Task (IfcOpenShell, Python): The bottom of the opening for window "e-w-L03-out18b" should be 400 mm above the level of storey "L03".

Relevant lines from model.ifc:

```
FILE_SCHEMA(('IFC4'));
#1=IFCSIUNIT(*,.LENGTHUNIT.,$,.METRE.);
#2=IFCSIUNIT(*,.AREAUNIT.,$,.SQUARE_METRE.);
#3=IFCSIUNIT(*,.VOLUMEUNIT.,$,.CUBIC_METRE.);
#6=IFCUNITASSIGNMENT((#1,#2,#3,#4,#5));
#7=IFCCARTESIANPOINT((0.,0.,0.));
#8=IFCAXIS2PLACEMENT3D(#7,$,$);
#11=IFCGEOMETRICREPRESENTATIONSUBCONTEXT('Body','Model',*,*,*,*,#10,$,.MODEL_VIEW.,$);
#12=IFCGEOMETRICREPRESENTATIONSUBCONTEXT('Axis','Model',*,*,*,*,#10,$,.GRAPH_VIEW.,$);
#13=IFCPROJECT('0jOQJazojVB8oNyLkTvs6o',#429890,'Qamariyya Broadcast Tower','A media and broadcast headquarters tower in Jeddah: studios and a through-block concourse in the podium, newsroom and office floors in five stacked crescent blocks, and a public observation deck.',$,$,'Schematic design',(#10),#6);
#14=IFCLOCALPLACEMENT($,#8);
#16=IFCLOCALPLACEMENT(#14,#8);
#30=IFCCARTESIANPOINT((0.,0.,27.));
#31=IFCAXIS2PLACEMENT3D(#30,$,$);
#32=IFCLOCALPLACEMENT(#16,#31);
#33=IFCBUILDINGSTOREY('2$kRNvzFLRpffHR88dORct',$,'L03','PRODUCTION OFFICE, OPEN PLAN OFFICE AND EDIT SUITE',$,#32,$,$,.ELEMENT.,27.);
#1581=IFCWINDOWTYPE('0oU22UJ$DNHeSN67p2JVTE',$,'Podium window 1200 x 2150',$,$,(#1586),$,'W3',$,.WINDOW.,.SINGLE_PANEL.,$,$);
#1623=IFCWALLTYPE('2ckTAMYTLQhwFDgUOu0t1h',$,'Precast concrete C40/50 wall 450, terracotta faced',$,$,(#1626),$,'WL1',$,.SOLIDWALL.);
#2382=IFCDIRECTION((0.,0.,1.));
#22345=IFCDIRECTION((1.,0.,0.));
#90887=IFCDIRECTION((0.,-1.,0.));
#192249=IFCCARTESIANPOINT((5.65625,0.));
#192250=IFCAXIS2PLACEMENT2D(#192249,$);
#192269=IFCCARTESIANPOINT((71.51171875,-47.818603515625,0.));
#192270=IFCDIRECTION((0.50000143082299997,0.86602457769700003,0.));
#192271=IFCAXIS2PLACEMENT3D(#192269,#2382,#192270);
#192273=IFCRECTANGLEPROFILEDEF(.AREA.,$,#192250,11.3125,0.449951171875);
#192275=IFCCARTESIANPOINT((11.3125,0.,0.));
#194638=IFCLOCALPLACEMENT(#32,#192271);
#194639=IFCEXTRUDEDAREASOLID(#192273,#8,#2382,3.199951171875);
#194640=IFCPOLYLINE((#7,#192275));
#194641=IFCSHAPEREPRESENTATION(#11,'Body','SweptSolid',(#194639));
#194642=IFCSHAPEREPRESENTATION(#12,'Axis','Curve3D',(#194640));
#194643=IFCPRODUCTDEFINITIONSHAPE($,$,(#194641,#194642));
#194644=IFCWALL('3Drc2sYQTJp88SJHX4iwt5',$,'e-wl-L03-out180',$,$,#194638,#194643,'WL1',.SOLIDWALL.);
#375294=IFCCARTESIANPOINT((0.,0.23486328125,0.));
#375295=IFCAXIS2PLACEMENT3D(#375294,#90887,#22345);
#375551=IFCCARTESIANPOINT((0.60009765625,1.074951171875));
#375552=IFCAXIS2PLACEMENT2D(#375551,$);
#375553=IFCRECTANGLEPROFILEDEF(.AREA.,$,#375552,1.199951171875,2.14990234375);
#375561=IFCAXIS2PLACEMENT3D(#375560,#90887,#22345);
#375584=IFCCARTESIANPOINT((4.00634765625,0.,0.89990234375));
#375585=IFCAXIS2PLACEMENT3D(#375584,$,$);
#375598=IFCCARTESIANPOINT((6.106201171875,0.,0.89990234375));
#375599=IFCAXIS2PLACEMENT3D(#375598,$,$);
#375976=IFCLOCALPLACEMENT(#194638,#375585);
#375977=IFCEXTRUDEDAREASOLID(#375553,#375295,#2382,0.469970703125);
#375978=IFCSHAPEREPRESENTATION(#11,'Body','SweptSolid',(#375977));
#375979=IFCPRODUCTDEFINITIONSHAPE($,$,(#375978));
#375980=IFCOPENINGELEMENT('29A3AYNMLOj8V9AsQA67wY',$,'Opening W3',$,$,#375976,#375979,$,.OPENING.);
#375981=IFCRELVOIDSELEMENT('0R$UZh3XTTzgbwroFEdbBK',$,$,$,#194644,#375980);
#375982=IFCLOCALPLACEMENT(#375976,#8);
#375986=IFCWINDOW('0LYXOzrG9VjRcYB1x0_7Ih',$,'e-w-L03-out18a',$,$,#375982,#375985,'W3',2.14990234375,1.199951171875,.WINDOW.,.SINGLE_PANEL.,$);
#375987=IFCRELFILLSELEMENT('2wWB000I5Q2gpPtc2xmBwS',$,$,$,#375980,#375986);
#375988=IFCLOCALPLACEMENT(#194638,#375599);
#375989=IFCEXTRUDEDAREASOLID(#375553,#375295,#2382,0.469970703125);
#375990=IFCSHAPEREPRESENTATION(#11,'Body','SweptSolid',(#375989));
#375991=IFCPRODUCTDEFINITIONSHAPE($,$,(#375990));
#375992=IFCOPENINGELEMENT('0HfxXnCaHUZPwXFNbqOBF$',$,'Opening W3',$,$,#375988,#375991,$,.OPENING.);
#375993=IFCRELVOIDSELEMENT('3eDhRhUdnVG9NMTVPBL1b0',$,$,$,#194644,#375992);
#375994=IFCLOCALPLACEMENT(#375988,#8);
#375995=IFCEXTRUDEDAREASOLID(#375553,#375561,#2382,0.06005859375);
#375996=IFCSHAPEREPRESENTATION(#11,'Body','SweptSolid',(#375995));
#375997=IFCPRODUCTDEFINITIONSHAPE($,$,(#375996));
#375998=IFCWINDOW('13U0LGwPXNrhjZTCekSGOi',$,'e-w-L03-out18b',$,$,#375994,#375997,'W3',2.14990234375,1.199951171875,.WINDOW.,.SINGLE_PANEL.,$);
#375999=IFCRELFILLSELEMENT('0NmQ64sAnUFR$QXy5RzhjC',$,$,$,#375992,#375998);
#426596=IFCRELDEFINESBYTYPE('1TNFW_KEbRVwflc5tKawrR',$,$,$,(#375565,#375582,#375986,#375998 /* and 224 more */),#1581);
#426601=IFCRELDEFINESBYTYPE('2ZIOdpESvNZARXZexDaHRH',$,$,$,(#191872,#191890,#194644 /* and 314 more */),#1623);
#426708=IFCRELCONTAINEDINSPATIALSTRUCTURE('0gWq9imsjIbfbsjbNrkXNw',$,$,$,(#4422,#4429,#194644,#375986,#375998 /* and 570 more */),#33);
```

```python
import numpy as np
import ifcopenshell
import ifcopenshell.api.geometry
import ifcopenshell.geom
import ifcopenshell.util.element
import ifcopenshell.util.placement
import ifcopenshell.util.shape
import ifcopenshell.util.unit

model = ifcopenshell.open("model.ifc")
unit_scale = ifcopenshell.util.unit.calculate_unit_scale(model)

window = model.by_id(375998)
opening = window.FillsVoids[0].RelatingOpeningElement
storey = ifcopenshell.util.element.get_container(window, ifc_class="IfcBuildingStorey")
level = ifcopenshell.util.placement.get_local_placement(storey.ObjectPlacement)[2, 3]

# The opening's origin need not be at the sill, so measure its lowest point.
shape = ifcopenshell.geom.create_shape(ifcopenshell.geom.settings(), opening)
bottom = ifcopenshell.util.shape.get_shape_bottom_elevation(shape, shape.geometry) / unit_scale
dz = level + 0.4 / unit_scale - bottom

shift = np.array([0.0, 0.0, dz])
# The window is placed relative to its opening, so it follows when the opening moves.
matrix = ifcopenshell.util.placement.get_local_placement(opening.ObjectPlacement)
matrix[:3, 3] += shift
ifcopenshell.api.geometry.edit_object_placement(
    model, product=opening, matrix=matrix, is_si=False, should_transform_children=True
)

print(f"moved by {dz * unit_scale:+.3f} m")

model.write("model_edited.ifc")
```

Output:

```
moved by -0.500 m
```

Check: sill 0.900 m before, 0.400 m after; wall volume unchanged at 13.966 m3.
